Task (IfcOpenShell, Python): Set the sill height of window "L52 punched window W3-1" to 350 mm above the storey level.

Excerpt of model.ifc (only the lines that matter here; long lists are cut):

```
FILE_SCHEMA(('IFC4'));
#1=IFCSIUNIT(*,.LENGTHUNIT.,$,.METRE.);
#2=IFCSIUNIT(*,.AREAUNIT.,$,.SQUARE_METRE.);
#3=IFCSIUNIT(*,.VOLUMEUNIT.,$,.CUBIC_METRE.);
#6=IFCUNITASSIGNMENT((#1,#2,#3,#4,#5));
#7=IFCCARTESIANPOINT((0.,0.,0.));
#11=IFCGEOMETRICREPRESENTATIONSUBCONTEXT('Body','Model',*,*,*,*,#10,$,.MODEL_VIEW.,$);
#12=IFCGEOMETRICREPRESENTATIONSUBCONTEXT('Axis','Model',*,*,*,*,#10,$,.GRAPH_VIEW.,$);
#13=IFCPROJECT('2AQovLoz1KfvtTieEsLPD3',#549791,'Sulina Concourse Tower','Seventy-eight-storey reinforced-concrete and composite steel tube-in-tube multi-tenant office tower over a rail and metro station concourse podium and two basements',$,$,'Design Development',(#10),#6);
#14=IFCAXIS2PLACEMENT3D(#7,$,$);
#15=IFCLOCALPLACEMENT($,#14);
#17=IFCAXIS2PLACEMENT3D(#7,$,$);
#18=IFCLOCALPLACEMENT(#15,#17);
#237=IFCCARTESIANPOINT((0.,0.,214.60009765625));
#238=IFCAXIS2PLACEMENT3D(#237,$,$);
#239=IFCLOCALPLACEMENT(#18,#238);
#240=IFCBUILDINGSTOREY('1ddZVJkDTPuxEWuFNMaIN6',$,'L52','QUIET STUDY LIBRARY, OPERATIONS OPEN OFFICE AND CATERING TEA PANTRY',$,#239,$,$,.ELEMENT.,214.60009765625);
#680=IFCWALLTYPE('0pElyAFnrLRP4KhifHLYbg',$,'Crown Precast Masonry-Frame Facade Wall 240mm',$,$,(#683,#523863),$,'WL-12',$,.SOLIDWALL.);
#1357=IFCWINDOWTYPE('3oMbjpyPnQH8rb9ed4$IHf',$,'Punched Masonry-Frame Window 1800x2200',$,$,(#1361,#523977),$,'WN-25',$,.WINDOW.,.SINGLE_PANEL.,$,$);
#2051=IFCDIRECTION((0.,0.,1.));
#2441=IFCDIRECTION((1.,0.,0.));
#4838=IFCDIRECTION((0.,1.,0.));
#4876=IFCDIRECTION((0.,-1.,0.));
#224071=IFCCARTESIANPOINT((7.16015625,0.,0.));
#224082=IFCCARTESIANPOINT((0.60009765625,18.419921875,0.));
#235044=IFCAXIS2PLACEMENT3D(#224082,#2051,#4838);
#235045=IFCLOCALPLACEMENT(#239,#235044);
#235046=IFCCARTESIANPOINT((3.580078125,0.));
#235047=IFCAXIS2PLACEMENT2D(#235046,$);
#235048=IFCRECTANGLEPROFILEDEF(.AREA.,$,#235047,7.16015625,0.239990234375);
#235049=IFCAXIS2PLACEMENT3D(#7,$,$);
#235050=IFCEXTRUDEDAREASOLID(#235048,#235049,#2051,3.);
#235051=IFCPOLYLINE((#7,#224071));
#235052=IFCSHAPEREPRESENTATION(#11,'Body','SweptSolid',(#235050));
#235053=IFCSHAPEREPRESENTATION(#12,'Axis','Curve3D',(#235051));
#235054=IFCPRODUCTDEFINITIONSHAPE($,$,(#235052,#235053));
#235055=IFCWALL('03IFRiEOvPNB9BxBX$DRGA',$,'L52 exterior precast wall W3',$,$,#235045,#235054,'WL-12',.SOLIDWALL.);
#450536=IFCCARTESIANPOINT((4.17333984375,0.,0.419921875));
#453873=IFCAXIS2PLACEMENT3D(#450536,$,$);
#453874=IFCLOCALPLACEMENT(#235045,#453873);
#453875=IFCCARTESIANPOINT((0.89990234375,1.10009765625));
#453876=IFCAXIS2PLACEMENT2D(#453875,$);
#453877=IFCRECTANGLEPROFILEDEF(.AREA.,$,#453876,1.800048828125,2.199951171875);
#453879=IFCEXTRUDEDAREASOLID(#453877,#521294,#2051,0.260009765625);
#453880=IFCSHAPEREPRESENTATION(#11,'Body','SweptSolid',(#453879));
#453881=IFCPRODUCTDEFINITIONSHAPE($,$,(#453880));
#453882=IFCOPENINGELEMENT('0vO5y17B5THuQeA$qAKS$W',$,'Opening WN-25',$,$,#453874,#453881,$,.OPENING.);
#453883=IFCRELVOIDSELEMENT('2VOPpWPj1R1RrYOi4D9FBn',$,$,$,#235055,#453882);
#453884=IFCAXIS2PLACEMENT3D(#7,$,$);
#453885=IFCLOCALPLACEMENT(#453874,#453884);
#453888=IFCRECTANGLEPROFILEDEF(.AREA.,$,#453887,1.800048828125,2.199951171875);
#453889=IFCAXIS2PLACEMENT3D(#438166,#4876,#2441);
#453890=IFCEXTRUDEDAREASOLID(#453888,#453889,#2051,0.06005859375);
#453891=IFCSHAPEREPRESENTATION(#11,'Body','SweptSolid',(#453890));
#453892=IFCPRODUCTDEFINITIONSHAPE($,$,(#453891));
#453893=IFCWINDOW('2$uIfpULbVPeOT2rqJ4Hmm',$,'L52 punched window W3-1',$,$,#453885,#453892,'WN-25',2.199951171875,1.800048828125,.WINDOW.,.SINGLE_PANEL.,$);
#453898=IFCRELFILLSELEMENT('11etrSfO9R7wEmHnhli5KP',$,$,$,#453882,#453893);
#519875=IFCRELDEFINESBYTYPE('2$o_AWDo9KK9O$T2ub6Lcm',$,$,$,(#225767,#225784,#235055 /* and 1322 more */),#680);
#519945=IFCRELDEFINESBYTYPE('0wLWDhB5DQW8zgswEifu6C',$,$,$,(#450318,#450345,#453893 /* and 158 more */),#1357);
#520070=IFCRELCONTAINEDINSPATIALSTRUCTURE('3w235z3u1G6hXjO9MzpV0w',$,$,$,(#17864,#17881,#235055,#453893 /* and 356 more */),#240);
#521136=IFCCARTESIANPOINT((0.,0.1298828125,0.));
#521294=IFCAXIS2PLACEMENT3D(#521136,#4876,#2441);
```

```python
import numpy as np
import ifcopenshell
import ifcopenshell.api.geometry
import ifcopenshell.geom
import ifcopenshell.util.element
import ifcopenshell.util.placement
import ifcopenshell.util.shape
import ifcopenshell.util.unit

model = ifcopenshell.open("model.ifc")
unit_scale = ifcopenshell.util.unit.calculate_unit_scale(model)

window = model.by_guid("2$uIfpULbVPeOT2rqJ4Hmm")
opening = window.FillsVoids[0].RelatingOpeningElement
storey = ifcopenshell.util.element.get_container(window, ifc_class="IfcBuildingStorey")
level = ifcopenshell.util.placement.get_local_placement(storey.ObjectPlacement)[2, 3]

# The opening's origin need not be at the sill, so measure its lowest point.
shape = ifcopenshell.geom.create_shape(ifcopenshell.geom.settings(), opening)
bottom = ifcopenshell.util.shape.get_shape_bottom_elevation(shape, shape.geometry) / unit_scale
dz = level + 0.35 - bottom

shift = np.array([0.0, 0.0, dz])
# The window is placed relative to its opening, so it follows when the opening moves.
matrix = ifcopenshell.util.placement.get_local_placement(opening.ObjectPlacement)
matrix[:3, 3] += shift
ifcopenshell.api.geometry.edit_object_placement(
    model, product=opening, matrix=matrix, is_si=False, should_transform_children=True
)

print(f"moved by {dz * unit_scale:+.3f} m")

model.write("model_edited.ifc")
```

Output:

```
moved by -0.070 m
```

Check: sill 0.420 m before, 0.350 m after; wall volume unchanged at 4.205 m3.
